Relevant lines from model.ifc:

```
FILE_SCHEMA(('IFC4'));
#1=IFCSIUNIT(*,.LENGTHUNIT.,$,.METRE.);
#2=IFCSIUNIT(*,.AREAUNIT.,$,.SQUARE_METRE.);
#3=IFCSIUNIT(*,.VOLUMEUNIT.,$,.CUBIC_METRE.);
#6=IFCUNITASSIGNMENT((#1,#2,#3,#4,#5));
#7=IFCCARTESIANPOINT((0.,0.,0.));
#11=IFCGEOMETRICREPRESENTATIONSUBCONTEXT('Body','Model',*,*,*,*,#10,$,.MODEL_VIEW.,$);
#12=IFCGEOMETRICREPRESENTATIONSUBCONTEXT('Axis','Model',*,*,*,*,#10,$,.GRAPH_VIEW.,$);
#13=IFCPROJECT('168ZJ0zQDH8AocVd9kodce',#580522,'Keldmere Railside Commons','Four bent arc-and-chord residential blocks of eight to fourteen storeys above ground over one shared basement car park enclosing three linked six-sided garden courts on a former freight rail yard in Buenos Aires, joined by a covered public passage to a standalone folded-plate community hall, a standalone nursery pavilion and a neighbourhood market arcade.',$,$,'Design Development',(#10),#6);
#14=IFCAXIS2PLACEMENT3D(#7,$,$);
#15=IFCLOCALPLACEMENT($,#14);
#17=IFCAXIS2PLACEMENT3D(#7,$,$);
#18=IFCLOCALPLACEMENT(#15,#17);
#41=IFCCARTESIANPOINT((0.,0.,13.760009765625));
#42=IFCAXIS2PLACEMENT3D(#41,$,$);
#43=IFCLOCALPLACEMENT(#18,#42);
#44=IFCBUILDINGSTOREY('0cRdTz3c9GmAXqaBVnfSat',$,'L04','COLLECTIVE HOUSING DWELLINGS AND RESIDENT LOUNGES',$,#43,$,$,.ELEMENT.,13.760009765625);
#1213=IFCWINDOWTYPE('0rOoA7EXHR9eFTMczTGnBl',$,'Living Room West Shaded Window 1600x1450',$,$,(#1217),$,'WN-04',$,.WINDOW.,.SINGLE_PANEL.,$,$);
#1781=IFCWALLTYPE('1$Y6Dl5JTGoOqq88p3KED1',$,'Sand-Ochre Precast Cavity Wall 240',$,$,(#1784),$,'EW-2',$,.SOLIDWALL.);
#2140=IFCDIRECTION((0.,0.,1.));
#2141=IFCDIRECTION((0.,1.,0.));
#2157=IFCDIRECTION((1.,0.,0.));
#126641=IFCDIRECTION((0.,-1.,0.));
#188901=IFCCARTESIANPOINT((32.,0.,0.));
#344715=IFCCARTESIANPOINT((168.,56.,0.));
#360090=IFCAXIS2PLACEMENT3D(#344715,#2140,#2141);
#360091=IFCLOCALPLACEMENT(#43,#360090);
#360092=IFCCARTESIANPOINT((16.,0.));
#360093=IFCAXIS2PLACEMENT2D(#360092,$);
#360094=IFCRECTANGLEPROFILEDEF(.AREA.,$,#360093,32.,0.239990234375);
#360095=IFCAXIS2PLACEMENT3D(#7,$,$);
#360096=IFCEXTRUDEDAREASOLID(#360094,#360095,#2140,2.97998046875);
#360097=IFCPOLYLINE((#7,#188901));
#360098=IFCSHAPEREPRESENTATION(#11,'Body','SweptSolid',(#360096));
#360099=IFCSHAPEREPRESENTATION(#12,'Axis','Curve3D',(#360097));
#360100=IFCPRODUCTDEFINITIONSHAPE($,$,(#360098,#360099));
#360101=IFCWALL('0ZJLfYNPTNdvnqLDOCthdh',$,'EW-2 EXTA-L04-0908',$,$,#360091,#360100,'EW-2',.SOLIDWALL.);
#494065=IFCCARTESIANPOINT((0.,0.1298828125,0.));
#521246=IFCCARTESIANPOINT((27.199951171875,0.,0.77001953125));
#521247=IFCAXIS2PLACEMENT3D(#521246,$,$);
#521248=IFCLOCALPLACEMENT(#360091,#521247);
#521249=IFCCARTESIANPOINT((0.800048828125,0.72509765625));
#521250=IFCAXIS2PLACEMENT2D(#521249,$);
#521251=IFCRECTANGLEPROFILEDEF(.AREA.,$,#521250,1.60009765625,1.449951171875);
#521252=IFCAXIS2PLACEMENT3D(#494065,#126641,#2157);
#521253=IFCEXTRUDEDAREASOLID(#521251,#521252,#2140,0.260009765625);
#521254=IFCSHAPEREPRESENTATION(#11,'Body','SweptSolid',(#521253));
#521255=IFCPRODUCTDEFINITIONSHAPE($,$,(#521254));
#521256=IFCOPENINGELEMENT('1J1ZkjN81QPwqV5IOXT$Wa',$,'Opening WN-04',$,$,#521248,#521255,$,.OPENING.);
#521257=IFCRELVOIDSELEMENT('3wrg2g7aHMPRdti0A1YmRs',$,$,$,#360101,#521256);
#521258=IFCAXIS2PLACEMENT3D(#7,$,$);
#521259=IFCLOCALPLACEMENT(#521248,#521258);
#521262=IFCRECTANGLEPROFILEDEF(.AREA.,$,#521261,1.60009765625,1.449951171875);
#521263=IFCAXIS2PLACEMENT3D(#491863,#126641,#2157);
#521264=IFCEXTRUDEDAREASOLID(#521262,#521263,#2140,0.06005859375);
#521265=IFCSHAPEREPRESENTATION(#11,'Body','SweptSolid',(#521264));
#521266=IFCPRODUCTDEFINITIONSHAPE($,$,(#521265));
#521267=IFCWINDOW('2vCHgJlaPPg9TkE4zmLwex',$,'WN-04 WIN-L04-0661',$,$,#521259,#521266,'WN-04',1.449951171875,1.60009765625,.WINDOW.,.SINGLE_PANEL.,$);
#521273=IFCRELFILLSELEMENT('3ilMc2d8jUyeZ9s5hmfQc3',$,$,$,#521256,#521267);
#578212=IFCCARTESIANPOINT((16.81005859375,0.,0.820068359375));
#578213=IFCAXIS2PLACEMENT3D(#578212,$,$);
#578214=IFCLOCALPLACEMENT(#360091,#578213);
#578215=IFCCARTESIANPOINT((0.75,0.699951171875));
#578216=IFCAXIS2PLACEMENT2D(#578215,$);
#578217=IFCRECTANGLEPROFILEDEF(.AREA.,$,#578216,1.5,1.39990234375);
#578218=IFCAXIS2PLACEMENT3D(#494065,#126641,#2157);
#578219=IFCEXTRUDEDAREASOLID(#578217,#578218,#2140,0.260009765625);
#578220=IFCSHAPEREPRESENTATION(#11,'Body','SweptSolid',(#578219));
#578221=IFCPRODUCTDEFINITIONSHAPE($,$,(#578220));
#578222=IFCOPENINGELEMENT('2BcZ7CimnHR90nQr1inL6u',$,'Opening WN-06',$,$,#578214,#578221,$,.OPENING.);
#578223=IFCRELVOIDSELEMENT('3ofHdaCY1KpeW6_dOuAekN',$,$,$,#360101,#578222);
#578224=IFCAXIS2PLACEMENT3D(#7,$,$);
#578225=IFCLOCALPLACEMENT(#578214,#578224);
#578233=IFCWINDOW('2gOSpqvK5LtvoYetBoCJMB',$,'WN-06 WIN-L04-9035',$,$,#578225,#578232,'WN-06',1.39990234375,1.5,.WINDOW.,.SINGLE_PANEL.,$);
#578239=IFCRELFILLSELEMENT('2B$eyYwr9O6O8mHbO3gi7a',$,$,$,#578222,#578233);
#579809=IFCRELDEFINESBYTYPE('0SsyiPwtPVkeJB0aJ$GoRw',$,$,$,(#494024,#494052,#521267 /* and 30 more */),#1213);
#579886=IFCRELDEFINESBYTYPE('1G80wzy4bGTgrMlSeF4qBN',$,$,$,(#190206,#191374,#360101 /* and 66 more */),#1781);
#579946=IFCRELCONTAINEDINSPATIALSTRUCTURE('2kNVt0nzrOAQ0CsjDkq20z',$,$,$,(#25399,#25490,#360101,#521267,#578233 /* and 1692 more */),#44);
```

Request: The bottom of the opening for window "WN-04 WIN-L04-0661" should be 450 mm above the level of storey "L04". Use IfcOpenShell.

```python
import numpy as np
import ifcopenshell
import ifcopenshell.api.geometry
import ifcopenshell.geom
import ifcopenshell.util.element
import ifcopenshell.util.placement
import ifcopenshell.util.shape
import ifcopenshell.util.unit

model = ifcopenshell.open("model.ifc")
unit_scale = ifcopenshell.util.unit.calculate_unit_scale(model)

window = model.by_id(521267)
opening = window.FillsVoids[0].RelatingOpeningElement
storey = ifcopenshell.util.element.get_container(window, ifc_class="IfcBuildingStorey")
level = ifcopenshell.util.placement.get_local_placement(storey.ObjectPlacement)[2, 3]

# The opening's origin need not be at the sill, so measure its lowest point.
shape = ifcopenshell.geom.create_shape(ifcopenshell.geom.settings(), opening)
bottom = ifcopenshell.util.shape.get_shape_bottom_elevation(shape, shape.geometry) / unit_scale
dz = level + 0.45 / unit_scale - bottom

shift = np.array([0.0, 0.0, dz])
# The window is placed relative to its opening, so it follows when the opening moves.
matrix = ifcopenshell.util.placement.get_local_placement(opening.ObjectPlacement)
matrix[:3, 3] += shift
ifcopenshell.api.geometry.edit_object_placement(
    model, product=opening, matrix=matrix, is_si=False, should_transform_children=True
)

print(f"moved by {dz * unit_scale:+.3f} m")

model.write("model-out.ifc")
```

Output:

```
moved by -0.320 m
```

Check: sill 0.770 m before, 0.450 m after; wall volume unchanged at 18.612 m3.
